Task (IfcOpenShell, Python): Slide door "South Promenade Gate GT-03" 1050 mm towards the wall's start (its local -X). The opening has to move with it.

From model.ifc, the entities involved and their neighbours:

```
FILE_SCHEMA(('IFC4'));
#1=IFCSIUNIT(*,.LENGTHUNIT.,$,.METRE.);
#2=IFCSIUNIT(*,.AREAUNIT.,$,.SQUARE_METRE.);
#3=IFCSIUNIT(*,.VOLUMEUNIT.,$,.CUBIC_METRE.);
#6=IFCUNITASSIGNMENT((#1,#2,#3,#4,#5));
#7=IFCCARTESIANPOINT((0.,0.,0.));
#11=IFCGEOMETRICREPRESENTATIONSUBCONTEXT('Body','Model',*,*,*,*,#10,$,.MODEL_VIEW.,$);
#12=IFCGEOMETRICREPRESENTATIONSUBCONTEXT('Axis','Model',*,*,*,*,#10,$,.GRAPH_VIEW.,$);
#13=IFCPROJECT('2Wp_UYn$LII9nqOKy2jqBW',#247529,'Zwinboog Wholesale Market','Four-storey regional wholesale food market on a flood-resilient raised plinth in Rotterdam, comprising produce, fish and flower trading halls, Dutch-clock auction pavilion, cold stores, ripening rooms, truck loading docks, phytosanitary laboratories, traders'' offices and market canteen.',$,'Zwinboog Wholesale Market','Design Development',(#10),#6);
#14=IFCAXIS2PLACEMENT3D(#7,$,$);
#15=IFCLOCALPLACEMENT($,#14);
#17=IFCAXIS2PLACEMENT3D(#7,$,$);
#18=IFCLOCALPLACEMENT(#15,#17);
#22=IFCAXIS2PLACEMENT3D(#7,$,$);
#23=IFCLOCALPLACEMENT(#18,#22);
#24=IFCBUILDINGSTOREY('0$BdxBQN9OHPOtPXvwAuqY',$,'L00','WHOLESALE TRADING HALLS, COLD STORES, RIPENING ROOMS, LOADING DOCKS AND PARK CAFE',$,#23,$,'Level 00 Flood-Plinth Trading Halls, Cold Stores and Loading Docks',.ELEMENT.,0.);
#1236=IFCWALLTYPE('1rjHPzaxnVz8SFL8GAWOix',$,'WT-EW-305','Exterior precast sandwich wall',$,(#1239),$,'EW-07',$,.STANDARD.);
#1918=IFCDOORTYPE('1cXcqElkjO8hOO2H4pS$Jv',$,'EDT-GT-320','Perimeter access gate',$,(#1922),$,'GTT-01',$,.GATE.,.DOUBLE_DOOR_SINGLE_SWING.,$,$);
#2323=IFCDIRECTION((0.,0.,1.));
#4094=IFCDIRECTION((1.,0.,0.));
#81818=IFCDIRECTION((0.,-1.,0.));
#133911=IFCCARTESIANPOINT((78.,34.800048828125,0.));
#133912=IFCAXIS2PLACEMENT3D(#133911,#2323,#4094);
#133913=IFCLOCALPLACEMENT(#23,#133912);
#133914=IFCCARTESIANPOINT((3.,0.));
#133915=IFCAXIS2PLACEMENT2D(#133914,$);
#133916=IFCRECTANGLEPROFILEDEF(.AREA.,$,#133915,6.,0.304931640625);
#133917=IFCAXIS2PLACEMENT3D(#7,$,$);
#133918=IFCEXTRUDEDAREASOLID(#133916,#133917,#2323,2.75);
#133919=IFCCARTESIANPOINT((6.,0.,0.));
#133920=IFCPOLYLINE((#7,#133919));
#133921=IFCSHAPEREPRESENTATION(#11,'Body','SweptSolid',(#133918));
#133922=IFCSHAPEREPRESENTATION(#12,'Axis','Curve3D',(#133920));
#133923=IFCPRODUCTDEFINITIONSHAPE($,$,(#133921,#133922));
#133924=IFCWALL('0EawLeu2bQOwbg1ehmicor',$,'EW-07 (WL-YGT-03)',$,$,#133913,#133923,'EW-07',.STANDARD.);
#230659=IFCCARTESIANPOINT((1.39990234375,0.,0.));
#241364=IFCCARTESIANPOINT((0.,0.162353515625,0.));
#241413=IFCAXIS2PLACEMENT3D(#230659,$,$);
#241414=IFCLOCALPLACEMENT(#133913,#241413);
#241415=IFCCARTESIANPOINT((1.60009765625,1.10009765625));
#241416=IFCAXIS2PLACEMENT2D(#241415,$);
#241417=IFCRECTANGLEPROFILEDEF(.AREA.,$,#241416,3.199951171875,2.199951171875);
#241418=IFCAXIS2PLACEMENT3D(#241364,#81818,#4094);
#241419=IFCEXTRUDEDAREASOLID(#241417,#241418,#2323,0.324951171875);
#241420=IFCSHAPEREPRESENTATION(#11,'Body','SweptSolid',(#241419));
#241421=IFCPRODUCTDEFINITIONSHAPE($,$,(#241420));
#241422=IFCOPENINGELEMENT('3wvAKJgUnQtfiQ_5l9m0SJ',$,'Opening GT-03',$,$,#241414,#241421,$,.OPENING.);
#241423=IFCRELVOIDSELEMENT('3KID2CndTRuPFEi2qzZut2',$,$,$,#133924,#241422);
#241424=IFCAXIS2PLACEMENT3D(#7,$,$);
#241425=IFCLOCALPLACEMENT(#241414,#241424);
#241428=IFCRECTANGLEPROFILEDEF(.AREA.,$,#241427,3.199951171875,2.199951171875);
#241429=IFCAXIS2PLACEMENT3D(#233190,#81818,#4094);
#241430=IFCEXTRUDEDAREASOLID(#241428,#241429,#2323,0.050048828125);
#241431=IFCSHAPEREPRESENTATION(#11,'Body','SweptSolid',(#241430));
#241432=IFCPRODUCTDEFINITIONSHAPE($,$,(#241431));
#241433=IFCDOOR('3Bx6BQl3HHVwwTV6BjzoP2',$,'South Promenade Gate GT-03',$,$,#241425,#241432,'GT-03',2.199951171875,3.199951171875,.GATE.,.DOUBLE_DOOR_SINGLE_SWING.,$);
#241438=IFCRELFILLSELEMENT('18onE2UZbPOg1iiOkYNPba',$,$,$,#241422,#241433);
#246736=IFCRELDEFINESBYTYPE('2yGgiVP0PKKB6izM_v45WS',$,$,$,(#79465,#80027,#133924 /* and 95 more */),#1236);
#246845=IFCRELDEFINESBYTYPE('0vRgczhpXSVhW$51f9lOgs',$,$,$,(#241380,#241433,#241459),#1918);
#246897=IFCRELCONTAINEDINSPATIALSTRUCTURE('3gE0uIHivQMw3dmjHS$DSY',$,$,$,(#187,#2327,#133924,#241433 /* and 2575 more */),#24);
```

```python
import ifcopenshell
import ifcopenshell.api.geometry
import ifcopenshell.util.placement
import ifcopenshell.util.unit

model = ifcopenshell.open("model.ifc")
unit_scale = ifcopenshell.util.unit.calculate_unit_scale(model)

door = model.by_id(241433)
opening = door.FillsVoids[0].RelatingOpeningElement
wall = opening.VoidsElements[0].RelatingBuildingElement

wall_matrix = ifcopenshell.util.placement.get_local_placement(wall.ObjectPlacement)
shift = wall_matrix[:3, 0] * -1.05 / unit_scale
before = ifcopenshell.util.placement.get_local_placement(door.ObjectPlacement)[:3, 3].copy()

# The door is placed relative to its opening, so it follows when the opening moves.
matrix = ifcopenshell.util.placement.get_local_placement(opening.ObjectPlacement)
matrix[:3, 3] += shift
ifcopenshell.api.geometry.edit_object_placement(
    model, product=opening, matrix=matrix, is_si=False, should_transform_children=True
)

after = ifcopenshell.util.placement.get_local_placement(door.ObjectPlacement)[:3, 3]
print("door moved by", (after - before).round(3) + 0.0)

model.write("model-out.ifc")
```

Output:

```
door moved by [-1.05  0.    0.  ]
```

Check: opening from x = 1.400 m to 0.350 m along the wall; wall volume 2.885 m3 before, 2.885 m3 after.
